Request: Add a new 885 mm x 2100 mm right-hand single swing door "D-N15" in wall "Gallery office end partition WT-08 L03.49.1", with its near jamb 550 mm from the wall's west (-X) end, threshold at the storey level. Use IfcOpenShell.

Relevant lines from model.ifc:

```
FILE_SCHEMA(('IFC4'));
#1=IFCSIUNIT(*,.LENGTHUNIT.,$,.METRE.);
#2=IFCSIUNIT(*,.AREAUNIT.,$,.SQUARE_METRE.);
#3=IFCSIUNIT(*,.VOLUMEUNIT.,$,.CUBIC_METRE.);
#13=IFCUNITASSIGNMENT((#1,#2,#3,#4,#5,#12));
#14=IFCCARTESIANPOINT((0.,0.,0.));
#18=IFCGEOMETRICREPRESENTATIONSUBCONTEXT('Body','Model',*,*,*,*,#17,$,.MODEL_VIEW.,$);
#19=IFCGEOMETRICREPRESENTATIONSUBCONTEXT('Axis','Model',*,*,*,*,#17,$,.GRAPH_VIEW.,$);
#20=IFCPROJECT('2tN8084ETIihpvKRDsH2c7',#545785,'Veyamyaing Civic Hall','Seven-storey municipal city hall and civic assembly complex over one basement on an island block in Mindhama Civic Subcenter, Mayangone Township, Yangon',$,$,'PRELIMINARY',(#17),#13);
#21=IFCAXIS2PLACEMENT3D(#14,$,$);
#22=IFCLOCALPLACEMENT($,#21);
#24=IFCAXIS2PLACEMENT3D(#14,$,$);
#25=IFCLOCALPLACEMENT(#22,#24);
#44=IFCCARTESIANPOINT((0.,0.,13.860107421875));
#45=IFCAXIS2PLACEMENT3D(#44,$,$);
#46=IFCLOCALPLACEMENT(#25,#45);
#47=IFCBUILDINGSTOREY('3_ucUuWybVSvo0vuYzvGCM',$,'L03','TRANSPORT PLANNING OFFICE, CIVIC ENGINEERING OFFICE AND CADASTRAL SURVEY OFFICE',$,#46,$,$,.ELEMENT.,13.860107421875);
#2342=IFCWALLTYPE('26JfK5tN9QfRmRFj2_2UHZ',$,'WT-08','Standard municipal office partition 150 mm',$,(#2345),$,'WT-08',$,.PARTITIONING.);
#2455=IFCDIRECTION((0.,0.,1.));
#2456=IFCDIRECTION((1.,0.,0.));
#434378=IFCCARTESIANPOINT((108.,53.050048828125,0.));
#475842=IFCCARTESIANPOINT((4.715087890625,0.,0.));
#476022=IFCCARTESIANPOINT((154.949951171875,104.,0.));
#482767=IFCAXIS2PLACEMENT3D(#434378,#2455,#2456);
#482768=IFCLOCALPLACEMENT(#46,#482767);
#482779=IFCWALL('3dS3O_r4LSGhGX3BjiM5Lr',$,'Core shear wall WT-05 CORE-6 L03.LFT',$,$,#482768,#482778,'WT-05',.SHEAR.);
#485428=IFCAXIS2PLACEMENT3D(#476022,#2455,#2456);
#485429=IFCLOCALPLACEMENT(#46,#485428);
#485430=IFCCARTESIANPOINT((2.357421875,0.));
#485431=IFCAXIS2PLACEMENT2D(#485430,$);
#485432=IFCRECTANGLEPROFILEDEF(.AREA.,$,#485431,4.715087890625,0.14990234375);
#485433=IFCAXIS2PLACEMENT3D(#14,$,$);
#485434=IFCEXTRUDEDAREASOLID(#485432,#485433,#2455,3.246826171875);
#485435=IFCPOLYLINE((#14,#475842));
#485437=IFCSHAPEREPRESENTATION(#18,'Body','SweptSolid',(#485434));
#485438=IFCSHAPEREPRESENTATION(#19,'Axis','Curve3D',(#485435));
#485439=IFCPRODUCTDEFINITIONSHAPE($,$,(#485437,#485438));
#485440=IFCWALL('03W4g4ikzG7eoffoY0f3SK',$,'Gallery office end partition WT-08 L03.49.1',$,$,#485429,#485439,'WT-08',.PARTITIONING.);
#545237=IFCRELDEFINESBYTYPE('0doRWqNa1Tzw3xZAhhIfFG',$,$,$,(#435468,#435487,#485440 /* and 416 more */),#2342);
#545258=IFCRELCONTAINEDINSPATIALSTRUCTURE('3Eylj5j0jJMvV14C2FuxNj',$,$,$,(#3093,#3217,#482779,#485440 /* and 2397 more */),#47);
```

```python
import numpy as np
import ifcopenshell
import ifcopenshell.api.feature
import ifcopenshell.api.geometry
import ifcopenshell.api.root
import ifcopenshell.api.spatial
import ifcopenshell.geom
import ifcopenshell.util.element
import ifcopenshell.util.placement
import ifcopenshell.util.representation
import ifcopenshell.util.shape
import ifcopenshell.util.unit

model = ifcopenshell.open("model.ifc")
unit_scale = ifcopenshell.util.unit.calculate_unit_scale(model)
settings = ifcopenshell.geom.settings()


def volume(element):
    """Net volume in cubic metres, openings subtracted."""
    shape = ifcopenshell.geom.create_shape(settings, element)
    return ifcopenshell.util.shape.get_volume(shape.geometry)


wall = model.by_guid("03W4g4ikzG7eoffoY0f3SK")
storey = ifcopenshell.util.element.get_container(wall, ifc_class="IfcBuildingStorey")
context = ifcopenshell.util.representation.get_context(model, "Model", "Body", "MODEL_VIEW")
before = volume(wall)

width, height, from_end, sill = 0.885, 2.1, 0.55, 0.0  # metres

# The wall runs along its own X axis, and the end named is its -X end.
wall_shape = ifcopenshell.geom.create_shape(settings, wall)
x, y, z = ifcopenshell.util.shape.get_vertices(wall_shape.geometry).T
start = x.min() + from_end
face, thickness = float(y.min()), float(y.max() - y.min())
wall_matrix = ifcopenshell.util.placement.get_local_placement(wall.ObjectPlacement)
level = ifcopenshell.util.placement.get_local_placement(storey.ObjectPlacement)[2, 3]


def in_wall(x, y):
    """Placement at x, y metres in the wall's axes, at sill height."""
    matrix = wall_matrix.copy()
    matrix[:, 3] = wall_matrix @ np.array([x / unit_scale, y / unit_scale, 0.0, 1.0])
    matrix[2, 3] = level + sill / unit_scale
    return matrix


# Opening: a box that overshoots both wall faces by 50 mm.
opening = ifcopenshell.api.root.create_entity(model, ifc_class="IfcOpeningElement", predefined_type="OPENING")
box = ifcopenshell.api.geometry.add_wall_representation(
    model, context=context, length=width, height=height, thickness=thickness + 0.1
)
ifcopenshell.api.geometry.assign_representation(model, product=opening, representation=box)
ifcopenshell.api.geometry.edit_object_placement(model, product=opening, matrix=in_wall(start, face - 0.05), is_si=False)
ifcopenshell.api.feature.add_feature(model, feature=opening, element=wall)

door = ifcopenshell.api.root.create_entity(model, ifc_class="IfcDoor", name="D-N15", predefined_type="DOOR")
door.OverallWidth, door.OverallHeight = width / unit_scale, height / unit_scale
door.OperationType = "SINGLE_SWING_RIGHT"
body = ifcopenshell.api.geometry.add_door_representation(
    model,
    context=context,
    overall_width=door.OverallWidth,
    overall_height=door.OverallHeight,
    operation_type="SINGLE_SWING_RIGHT",
    lining_properties={"LiningDepth": thickness / unit_scale, "ThresholdDepth": thickness / unit_scale},
)
ifcopenshell.api.geometry.assign_representation(model, product=door, representation=body)
ifcopenshell.api.spatial.assign_container(model, products=[door], relating_structure=storey)
ifcopenshell.api.feature.add_filling(model, opening=opening, element=door)

# The lining spans the wall, so the door starts at the wall face.
ifcopenshell.api.geometry.edit_object_placement(model, product=door, matrix=in_wall(start, face), is_si=False)

after = volume(wall)

print(f"wall volume {before:.3f} -> {after:.3f} m3")

model.write("model_edited.ifc")
```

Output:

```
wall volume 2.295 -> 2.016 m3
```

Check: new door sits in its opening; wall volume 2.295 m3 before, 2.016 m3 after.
